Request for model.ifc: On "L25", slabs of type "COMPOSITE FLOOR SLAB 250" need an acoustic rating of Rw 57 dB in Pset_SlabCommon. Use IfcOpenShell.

First a look at what the model holds.

```python
import ifcopenshell
import ifcopenshell.util.element

model = ifcopenshell.open("model.ifc")
print(model.schema)
storey = next(s for s in model.by_type("IfcBuildingStorey") if s.Name == "L25")
slabs = [e for e in ifcopenshell.util.element.get_decomposition(storey) if e.is_a("IfcSlab")]
seen = {}
for e in slabs:
    element_type = ifcopenshell.util.element.get_type(e)
    key = (element_type.Name if element_type != e and element_type else None, ifcopenshell.util.element.get_pset(e, "Pset_SlabCommon", "AcousticRating"))
    seen[key] = seen.get(key, 0) + 1
for (name, value), count in sorted(seen.items(), key=str):
    print(count, "x", name, "|", value)
```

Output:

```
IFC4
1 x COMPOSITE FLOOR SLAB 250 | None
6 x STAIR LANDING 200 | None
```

```python
import ifcopenshell
import ifcopenshell.api.pset
import ifcopenshell.util.element

model = ifcopenshell.open("model.ifc")

storey = next(s for s in model.by_type("IfcBuildingStorey") if s.Name == "L25")
slabs = [e for e in ifcopenshell.util.element.get_decomposition(storey) if e.is_a("IfcSlab")]

count = 0
for e in slabs:
    element_type = ifcopenshell.util.element.get_type(e)
    if element_type in (None, e) or element_type.Name != "COMPOSITE FLOOR SLAB 250":
        continue
    # add_pset returns the element's existing set when there is one.
    pset = ifcopenshell.api.pset.add_pset(model, product=e, name="Pset_SlabCommon")
    ifcopenshell.api.pset.edit_pset(model, pset=pset, properties={"AcousticRating": "Rw 57 dB"})
    count += 1

print(count, "slabs updated")

model.write("model_updated.ifc")
```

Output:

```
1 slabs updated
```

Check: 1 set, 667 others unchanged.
